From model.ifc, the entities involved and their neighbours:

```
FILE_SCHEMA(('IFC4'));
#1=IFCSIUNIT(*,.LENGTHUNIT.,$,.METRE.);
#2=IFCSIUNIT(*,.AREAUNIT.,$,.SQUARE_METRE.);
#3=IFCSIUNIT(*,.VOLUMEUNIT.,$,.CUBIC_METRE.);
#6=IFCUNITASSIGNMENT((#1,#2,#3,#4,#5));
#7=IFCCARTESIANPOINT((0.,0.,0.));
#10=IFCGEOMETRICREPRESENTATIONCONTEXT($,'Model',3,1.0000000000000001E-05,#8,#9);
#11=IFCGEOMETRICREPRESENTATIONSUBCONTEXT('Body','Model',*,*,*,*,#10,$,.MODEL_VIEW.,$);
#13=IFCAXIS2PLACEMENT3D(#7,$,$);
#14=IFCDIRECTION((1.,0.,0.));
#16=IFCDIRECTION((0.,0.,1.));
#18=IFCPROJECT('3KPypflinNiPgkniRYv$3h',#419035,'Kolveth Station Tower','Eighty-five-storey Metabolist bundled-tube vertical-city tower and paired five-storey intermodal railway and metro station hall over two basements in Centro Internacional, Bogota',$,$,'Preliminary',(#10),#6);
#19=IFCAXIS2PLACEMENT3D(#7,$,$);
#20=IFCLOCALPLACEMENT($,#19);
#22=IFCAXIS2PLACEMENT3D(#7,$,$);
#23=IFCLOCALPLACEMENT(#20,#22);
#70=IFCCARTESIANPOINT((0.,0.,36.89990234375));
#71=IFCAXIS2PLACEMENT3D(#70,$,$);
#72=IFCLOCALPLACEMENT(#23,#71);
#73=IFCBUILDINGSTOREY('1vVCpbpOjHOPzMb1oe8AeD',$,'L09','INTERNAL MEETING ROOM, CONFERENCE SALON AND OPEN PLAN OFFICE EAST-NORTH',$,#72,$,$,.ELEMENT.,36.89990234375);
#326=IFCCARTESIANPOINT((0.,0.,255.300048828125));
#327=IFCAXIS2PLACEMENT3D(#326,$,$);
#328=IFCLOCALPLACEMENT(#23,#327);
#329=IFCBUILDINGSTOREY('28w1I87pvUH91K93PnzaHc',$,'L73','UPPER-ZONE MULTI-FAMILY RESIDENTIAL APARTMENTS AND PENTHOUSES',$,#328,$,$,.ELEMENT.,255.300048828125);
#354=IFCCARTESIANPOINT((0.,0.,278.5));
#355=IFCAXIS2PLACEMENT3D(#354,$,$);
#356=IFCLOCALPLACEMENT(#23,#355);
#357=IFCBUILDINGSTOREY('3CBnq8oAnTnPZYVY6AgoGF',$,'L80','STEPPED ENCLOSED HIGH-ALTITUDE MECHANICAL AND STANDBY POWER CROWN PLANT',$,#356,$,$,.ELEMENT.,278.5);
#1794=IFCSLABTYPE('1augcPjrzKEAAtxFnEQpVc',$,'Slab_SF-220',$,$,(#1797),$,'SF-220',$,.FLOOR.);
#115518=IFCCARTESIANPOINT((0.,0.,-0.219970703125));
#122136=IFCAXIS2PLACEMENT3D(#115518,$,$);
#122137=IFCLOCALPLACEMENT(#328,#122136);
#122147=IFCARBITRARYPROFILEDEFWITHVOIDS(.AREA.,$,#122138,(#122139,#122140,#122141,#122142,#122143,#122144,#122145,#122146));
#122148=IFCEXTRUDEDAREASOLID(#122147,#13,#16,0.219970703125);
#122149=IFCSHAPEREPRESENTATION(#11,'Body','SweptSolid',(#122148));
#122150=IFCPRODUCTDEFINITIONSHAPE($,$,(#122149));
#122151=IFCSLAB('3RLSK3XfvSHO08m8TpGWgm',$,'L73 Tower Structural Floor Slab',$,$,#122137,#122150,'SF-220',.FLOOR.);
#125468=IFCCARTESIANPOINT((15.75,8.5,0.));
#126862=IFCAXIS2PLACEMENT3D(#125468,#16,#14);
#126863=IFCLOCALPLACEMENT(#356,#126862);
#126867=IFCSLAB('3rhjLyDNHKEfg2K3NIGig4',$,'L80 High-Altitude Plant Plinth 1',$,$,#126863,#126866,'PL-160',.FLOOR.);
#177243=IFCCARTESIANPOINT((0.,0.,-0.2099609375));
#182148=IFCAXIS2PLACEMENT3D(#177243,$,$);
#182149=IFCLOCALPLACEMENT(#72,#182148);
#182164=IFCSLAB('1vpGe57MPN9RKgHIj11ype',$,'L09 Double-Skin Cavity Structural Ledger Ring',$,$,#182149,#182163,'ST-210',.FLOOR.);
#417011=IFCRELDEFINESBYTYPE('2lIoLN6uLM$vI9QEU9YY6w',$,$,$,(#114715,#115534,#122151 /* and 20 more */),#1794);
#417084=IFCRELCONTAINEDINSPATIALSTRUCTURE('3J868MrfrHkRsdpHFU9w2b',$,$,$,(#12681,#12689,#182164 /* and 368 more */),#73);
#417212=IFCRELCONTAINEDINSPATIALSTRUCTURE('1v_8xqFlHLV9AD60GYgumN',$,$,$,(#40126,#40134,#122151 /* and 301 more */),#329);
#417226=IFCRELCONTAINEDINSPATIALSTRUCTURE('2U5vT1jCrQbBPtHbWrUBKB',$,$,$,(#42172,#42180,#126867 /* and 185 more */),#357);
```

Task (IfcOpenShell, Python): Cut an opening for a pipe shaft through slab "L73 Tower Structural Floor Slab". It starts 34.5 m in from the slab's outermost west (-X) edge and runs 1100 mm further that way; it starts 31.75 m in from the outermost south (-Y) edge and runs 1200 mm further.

```python
import numpy as np
import ifcopenshell
import ifcopenshell.api.feature
import ifcopenshell.api.geometry
import ifcopenshell.api.root
import ifcopenshell.geom
import ifcopenshell.util.placement
import ifcopenshell.util.representation
import ifcopenshell.util.shape
import ifcopenshell.util.unit

model = ifcopenshell.open("model.ifc")
unit_scale = ifcopenshell.util.unit.calculate_unit_scale(model)
settings = ifcopenshell.geom.settings()


def volume(element):
    """Net volume in cubic metres, openings subtracted."""
    shape = ifcopenshell.geom.create_shape(settings, element)
    return ifcopenshell.util.shape.get_volume(shape.geometry)


slab = model.by_guid("3RLSK3XfvSHO08m8TpGWgm")
before = volume(slab)

# Extent in the slab's own axes, in metres. The edges named are its -X and -Y sides.
slab_shape = ifcopenshell.geom.create_shape(settings, slab)
vertices = ifcopenshell.util.shape.get_vertices(slab_shape.geometry)
x_min, y_min, bottom = vertices.min(axis=0)
top = vertices[:, 2].max()

opening = ifcopenshell.api.root.create_entity(model, ifc_class="IfcOpeningElement", name="Pipe shaft opening", predefined_type="OPENING")
context = ifcopenshell.util.representation.get_context(model, "Model", "Body", "MODEL_VIEW")
width, depth = 1.1, 1.2
outline = [(0.0, 0.0), (width, 0.0), (width, depth), (0.0, depth), (0.0, 0.0)]
# Overshoot both faces by 50 mm so the cut is clean.
shape = ifcopenshell.api.geometry.add_slab_representation(
    model, context=context, depth=top - bottom + 0.1, polyline=outline
)
ifcopenshell.api.geometry.assign_representation(model, product=opening, representation=shape)

matrix = ifcopenshell.util.placement.get_local_placement(slab.ObjectPlacement)
matrix[:, 3] = matrix @ np.append(np.array([x_min + 34.5, y_min + 31.75, bottom - 0.05]) / unit_scale, 1.0)
ifcopenshell.api.geometry.edit_object_placement(model, product=opening, matrix=matrix, is_si=False)
ifcopenshell.api.feature.add_feature(model, feature=opening, element=slab)

after = volume(slab)

print(f"slab volume {before:.3f} -> {after:.3f} m3")

model.write("model_v2.ifc")
```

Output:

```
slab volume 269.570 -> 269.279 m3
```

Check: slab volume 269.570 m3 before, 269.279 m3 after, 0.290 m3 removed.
